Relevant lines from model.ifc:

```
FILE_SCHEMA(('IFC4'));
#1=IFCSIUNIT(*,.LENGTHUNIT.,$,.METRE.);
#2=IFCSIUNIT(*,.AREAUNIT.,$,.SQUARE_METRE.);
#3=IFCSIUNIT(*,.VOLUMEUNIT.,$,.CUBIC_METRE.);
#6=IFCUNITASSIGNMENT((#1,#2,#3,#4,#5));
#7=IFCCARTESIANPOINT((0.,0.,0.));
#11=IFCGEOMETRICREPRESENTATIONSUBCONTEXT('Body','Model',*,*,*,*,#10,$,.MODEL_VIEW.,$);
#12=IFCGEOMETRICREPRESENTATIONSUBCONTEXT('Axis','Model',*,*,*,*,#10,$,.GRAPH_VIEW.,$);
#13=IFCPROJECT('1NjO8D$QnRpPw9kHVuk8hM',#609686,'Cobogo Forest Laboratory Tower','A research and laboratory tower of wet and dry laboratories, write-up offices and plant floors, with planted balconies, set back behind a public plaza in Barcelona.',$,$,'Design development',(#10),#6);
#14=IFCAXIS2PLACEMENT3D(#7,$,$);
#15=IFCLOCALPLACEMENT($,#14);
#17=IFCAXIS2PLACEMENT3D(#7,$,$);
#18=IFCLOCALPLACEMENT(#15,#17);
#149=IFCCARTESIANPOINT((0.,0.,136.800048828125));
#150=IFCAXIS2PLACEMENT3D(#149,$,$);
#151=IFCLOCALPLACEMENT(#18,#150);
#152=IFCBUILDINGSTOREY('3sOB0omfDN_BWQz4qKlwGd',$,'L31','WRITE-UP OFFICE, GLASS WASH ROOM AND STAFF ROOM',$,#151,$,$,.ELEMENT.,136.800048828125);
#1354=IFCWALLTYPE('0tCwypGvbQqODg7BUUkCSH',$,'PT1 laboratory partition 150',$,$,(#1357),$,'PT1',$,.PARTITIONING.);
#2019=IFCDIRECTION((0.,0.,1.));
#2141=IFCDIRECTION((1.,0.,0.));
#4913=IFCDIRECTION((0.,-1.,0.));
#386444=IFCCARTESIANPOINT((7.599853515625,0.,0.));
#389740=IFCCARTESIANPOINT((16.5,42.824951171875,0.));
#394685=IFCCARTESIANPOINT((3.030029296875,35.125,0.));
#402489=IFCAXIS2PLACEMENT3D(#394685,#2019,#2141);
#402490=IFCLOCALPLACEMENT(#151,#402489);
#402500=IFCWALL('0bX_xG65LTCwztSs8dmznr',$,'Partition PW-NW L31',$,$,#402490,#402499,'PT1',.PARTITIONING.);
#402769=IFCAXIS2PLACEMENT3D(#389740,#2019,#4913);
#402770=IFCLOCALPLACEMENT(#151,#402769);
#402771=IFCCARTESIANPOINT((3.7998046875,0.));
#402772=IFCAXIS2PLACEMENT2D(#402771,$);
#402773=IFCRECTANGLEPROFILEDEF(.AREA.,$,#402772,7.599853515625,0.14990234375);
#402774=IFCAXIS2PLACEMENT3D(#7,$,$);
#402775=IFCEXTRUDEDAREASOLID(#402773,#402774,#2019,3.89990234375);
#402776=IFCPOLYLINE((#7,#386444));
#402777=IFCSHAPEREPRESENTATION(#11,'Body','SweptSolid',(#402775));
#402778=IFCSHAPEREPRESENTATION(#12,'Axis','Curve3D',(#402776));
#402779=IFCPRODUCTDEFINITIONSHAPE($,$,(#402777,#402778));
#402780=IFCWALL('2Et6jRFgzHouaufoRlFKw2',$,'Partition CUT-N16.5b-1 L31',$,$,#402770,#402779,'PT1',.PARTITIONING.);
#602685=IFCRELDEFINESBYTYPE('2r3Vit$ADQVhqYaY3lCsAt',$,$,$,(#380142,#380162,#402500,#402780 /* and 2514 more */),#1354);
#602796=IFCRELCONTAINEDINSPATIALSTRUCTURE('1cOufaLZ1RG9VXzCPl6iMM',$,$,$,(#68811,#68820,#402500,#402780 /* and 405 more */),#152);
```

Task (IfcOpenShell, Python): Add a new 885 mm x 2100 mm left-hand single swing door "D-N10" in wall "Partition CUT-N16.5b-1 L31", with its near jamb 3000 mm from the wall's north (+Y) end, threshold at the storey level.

```python
import numpy as np
import ifcopenshell
import ifcopenshell.api.feature
import ifcopenshell.api.geometry
import ifcopenshell.api.root
import ifcopenshell.api.spatial
import ifcopenshell.geom
import ifcopenshell.util.element
import ifcopenshell.util.placement
import ifcopenshell.util.representation
import ifcopenshell.util.shape
import ifcopenshell.util.unit

model = ifcopenshell.open("model.ifc")
unit_scale = ifcopenshell.util.unit.calculate_unit_scale(model)
settings = ifcopenshell.geom.settings()


def volume(element):
    """Net volume in cubic metres, openings subtracted."""
    shape = ifcopenshell.geom.create_shape(settings, element)
    return ifcopenshell.util.shape.get_volume(shape.geometry)


wall = model.by_guid("2Et6jRFgzHouaufoRlFKw2")
storey = ifcopenshell.util.element.get_container(wall, ifc_class="IfcBuildingStorey")
context = ifcopenshell.util.representation.get_context(model, "Model", "Body", "MODEL_VIEW")
before = volume(wall)

width, height, from_end, sill = 0.885, 2.1, 3, 0.0  # metres

# The wall runs along its own X axis, and the end named is its -X end.
wall_shape = ifcopenshell.geom.create_shape(settings, wall)
x, y, z = ifcopenshell.util.shape.get_vertices(wall_shape.geometry).T
start = x.min() + from_end
face, thickness = float(y.min()), float(y.max() - y.min())
wall_matrix = ifcopenshell.util.placement.get_local_placement(wall.ObjectPlacement)
level = ifcopenshell.util.placement.get_local_placement(storey.ObjectPlacement)[2, 3]


def in_wall(x, y):
    """Placement at x, y metres in the wall's axes, at sill height."""
    matrix = wall_matrix.copy()
    matrix[:, 3] = wall_matrix @ np.array([x / unit_scale, y / unit_scale, 0.0, 1.0])
    matrix[2, 3] = level + sill / unit_scale
    return matrix


# Opening: a box that overshoots both wall faces by 50 mm.
opening = ifcopenshell.api.root.create_entity(model, ifc_class="IfcOpeningElement", predefined_type="OPENING")
box = ifcopenshell.api.geometry.add_wall_representation(
    model, context=context, length=width, height=height, thickness=thickness + 0.1
)
ifcopenshell.api.geometry.assign_representation(model, product=opening, representation=box)
ifcopenshell.api.geometry.edit_object_placement(model, product=opening, matrix=in_wall(start, face - 0.05), is_si=False)
ifcopenshell.api.feature.add_feature(model, feature=opening, element=wall)

door = ifcopenshell.api.root.create_entity(model, ifc_class="IfcDoor", name="D-N10", predefined_type="DOOR")
door.OverallWidth, door.OverallHeight = width / unit_scale, height / unit_scale
door.OperationType = "SINGLE_SWING_LEFT"
body = ifcopenshell.api.geometry.add_door_representation(
    model,
    context=context,
    overall_width=door.OverallWidth,
    overall_height=door.OverallHeight,
    operation_type="SINGLE_SWING_LEFT",
    lining_properties={"LiningDepth": thickness / unit_scale, "ThresholdDepth": thickness / unit_scale},
)
ifcopenshell.api.geometry.assign_representation(model, product=door, representation=body)
ifcopenshell.api.spatial.assign_container(model, products=[door], relating_structure=storey)
ifcopenshell.api.feature.add_filling(model, opening=opening, element=door)

# The lining spans the wall, so the door starts at the wall face.
ifcopenshell.api.geometry.edit_object_placement(model, product=door, matrix=in_wall(start, face), is_si=False)

after = volume(wall)

print(f"wall volume {before:.3f} -> {after:.3f} m3")

model.write("model_updated.ifc")
```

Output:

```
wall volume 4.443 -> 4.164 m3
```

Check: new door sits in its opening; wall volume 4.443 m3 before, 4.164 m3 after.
